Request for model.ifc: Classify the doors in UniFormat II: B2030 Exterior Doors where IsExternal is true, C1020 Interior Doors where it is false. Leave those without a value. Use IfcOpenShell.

First a look at what the model holds.

```python
import ifcopenshell
import ifcopenshell.util.element

model = ifcopenshell.open("model.ifc")
print(model.schema)
print("classifications:", [c.Name for c in model.by_type("IfcClassification")])
values = [ifcopenshell.util.element.get_pset(e, "Pset_DoorCommon", "IsExternal") for e in model.by_type("IfcDoor")]
for value in (True, False, None):
    print("IsExternal", value, values.count(value))
```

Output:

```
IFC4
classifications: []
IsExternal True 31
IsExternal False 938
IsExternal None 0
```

```python
import ifcopenshell
import ifcopenshell.api.classification
import ifcopenshell.util.element

model = ifcopenshell.open("model.ifc")

system = ifcopenshell.api.classification.add_classification(model, classification="UniFormat II")

doors = model.by_type("IfcDoor")
external = {e: ifcopenshell.util.element.get_pset(e, "Pset_DoorCommon", "IsExternal") for e in doors}
for flag, code, name in ((True, "B2030", "Exterior Doors"), (False, "C1020", "Interior Doors")):
    products = [e for e in doors if external[e] is flag]
    ifcopenshell.api.classification.add_reference(
        model, products=products, classification=system, identification=code, name=name
    )
    print(code, len(products))

model.write("model_rev.ifc")
```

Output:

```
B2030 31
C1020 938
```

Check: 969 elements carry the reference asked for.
